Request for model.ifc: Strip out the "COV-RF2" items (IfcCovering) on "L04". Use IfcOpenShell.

First a look at what the model holds.

```python
import ifcopenshell
import ifcopenshell.util.element

model = ifcopenshell.open("model.ifc")
print(model.schema)
storey = next(s for s in model.by_type("IfcBuildingStorey") if s.Name == "L04")
coverings = [e for e in ifcopenshell.util.element.get_decomposition(storey) if e.is_a("IfcCovering")]
seen = {}
for e in coverings:
    element_type = ifcopenshell.util.element.get_type(e)
    name = element_type.Name if element_type not in (None, e) else None
    seen[name] = seen.get(name, 0) + 1
for name, count in sorted(seen.items(), key=str):
    print(count, "x", name)
```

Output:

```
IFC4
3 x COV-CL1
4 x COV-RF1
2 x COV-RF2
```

```python
import ifcopenshell
import ifcopenshell.api.root
import ifcopenshell.util.element

model = ifcopenshell.open("model.ifc")

storey = next(s for s in model.by_type("IfcBuildingStorey") if s.Name == "L04")
coverings = [e for e in ifcopenshell.util.element.get_decomposition(storey) if e.is_a("IfcCovering")]
targets = [e for e in coverings if (t := ifcopenshell.util.element.get_type(e)) not in (None, e) and t.Name == "COV-RF2"]

for e in targets:
    ifcopenshell.api.root.remove_product(model, product=e)
print(len(targets), "removed")

model.write("model_edited.ifc")
```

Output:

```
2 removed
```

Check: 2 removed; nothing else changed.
